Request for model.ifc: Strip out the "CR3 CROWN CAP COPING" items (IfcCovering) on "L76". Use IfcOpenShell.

First a look at what the model holds.

```python
import ifcopenshell
import ifcopenshell.util.element

model = ifcopenshell.open("model.ifc")
print(model.schema)
storey = next(s for s in model.by_type("IfcBuildingStorey") if s.Name == "L76")
coverings = [e for e in ifcopenshell.util.element.get_decomposition(storey) if e.is_a("IfcCovering")]
seen = {}
for e in coverings:
    element_type = ifcopenshell.util.element.get_type(e)
    name = element_type.Name if element_type not in (None, e) else None
    seen[name] = seen.get(name, 0) + 1
for name, count in sorted(seen.items(), key=str):
    print(count, "x", name)
```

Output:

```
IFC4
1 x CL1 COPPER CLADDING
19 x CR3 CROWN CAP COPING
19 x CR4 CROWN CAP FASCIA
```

```python
import ifcopenshell
import ifcopenshell.api.root
import ifcopenshell.util.element

model = ifcopenshell.open("model.ifc")

storey = next(s for s in model.by_type("IfcBuildingStorey") if s.Name == "L76")
coverings = [e for e in ifcopenshell.util.element.get_decomposition(storey) if e.is_a("IfcCovering")]
targets = [e for e in coverings if (t := ifcopenshell.util.element.get_type(e)) not in (None, e) and t.Name == "CR3 CROWN CAP COPING"]

for e in targets:
    ifcopenshell.api.root.remove_product(model, product=e)
print(len(targets), "removed")

model.write("model_rev.ifc")
```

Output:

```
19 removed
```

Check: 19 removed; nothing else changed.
